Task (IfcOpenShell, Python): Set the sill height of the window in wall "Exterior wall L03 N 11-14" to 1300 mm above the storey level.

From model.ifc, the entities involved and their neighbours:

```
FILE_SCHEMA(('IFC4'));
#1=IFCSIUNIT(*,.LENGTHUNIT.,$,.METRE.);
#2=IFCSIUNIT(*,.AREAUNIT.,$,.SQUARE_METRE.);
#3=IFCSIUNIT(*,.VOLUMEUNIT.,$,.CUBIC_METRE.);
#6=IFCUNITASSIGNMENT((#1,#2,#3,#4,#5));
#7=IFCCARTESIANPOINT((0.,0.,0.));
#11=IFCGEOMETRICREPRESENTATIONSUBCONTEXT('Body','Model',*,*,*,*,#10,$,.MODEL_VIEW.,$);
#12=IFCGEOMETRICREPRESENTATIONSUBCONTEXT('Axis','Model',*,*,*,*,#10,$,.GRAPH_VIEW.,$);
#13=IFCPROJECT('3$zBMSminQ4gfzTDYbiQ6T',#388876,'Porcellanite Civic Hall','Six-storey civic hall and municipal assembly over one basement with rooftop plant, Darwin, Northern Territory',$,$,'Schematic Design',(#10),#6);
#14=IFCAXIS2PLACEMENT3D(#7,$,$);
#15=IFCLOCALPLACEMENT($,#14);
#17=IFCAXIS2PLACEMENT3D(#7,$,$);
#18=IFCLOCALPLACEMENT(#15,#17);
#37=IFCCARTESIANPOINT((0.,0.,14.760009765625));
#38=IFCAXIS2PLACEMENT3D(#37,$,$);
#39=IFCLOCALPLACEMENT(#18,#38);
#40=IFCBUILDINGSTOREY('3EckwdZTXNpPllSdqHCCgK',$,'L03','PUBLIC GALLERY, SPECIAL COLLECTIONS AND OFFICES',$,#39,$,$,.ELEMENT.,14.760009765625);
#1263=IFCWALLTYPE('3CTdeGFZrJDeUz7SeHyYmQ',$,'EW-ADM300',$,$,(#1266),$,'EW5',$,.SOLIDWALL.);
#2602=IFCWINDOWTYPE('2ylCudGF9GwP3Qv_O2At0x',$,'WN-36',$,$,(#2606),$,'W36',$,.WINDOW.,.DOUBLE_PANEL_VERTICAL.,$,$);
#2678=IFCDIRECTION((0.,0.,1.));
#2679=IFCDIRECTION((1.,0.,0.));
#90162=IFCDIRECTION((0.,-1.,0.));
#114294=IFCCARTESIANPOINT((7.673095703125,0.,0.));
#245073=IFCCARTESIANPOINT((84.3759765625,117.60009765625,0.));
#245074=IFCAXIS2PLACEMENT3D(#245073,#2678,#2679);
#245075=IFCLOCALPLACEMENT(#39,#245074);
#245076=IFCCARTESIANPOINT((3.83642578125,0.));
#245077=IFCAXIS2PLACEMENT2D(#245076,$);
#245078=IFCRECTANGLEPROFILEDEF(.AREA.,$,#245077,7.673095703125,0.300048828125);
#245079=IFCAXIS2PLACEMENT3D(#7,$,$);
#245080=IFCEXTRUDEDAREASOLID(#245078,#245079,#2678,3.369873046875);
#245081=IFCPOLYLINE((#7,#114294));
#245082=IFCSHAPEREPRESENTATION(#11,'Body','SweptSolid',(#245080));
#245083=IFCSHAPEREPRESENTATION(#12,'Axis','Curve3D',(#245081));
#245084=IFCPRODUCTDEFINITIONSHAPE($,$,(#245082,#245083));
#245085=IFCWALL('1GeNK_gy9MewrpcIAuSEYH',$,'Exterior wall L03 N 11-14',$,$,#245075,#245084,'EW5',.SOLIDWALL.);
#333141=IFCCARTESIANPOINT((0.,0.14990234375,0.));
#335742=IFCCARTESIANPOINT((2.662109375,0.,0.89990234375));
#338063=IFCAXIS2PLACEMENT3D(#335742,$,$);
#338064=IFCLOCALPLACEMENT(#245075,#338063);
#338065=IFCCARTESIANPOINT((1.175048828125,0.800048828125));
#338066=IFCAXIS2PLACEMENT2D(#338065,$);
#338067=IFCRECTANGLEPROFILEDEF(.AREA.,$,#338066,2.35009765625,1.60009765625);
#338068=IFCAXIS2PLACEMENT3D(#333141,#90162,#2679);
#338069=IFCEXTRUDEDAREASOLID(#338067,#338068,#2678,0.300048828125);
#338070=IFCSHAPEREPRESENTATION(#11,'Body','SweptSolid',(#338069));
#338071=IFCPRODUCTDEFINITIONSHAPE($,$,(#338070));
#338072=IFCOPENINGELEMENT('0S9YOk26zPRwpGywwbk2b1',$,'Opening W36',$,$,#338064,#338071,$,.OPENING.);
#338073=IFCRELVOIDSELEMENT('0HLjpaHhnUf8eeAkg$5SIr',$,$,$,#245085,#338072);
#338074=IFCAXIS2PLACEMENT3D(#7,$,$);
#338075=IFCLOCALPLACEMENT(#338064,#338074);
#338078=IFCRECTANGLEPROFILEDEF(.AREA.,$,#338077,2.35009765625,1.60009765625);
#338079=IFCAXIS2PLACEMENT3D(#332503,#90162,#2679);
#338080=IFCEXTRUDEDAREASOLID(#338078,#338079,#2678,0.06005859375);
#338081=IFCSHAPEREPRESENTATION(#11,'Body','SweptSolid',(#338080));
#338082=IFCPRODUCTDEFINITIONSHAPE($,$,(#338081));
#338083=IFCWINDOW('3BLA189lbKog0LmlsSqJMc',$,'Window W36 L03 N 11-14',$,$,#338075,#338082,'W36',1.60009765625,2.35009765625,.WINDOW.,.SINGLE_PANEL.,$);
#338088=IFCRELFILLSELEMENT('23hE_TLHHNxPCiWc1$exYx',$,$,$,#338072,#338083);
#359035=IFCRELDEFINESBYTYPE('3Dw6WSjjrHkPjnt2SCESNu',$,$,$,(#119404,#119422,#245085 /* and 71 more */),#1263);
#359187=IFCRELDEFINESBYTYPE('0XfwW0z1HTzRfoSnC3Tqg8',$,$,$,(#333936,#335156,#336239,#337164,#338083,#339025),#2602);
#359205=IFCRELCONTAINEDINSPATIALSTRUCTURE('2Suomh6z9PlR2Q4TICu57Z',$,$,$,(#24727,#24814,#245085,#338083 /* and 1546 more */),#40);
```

```python
import numpy as np
import ifcopenshell
import ifcopenshell.api.geometry
import ifcopenshell.geom
import ifcopenshell.util.element
import ifcopenshell.util.placement
import ifcopenshell.util.shape
import ifcopenshell.util.unit

model = ifcopenshell.open("model.ifc")
unit_scale = ifcopenshell.util.unit.calculate_unit_scale(model)

window = model.by_id(338083)
opening = window.FillsVoids[0].RelatingOpeningElement
storey = ifcopenshell.util.element.get_container(window, ifc_class="IfcBuildingStorey")
level = ifcopenshell.util.placement.get_local_placement(storey.ObjectPlacement)[2, 3]

# The opening's origin need not be at the sill, so measure its lowest point.
shape = ifcopenshell.geom.create_shape(ifcopenshell.geom.settings(), opening)
bottom = ifcopenshell.util.shape.get_shape_bottom_elevation(shape, shape.geometry) / unit_scale
dz = level + 1.3 - bottom

shift = np.array([0.0, 0.0, dz])
# The window is placed relative to its opening, so it follows when the opening moves.
matrix = ifcopenshell.util.placement.get_local_placement(opening.ObjectPlacement)
matrix[:3, 3] += shift
ifcopenshell.api.geometry.edit_object_placement(
    model, product=opening, matrix=matrix, is_si=False, should_transform_children=True
)

print(f"moved by {dz * unit_scale:+.3f} m")

model.write("model_rev.ifc")
```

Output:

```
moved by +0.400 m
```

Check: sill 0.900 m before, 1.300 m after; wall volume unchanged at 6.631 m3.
